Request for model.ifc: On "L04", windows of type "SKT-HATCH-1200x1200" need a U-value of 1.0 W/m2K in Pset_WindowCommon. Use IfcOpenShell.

First a look at what the model holds.

```python
import ifcopenshell
import ifcopenshell.util.element

model = ifcopenshell.open("model.ifc")
print(model.schema)
storey = next(s for s in model.by_type("IfcBuildingStorey") if s.Name == "L04")
windows = [e for e in ifcopenshell.util.element.get_decomposition(storey) if e.is_a("IfcWindow")]
seen = {}
for e in windows:
    element_type = ifcopenshell.util.element.get_type(e)
    key = (element_type.Name if element_type != e and element_type else None, ifcopenshell.util.element.get_pset(e, "Pset_WindowCommon", "ThermalTransmittance"))
    seen[key] = seen.get(key, 0) + 1
for (name, value), count in sorted(seen.items(), key=str):
    print(count, "x", name, "|", value)
```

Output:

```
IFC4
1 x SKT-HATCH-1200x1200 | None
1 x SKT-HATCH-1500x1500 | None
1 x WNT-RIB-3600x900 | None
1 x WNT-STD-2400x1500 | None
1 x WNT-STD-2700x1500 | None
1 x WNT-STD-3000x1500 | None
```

```python
import ifcopenshell
import ifcopenshell.api.pset
import ifcopenshell.util.element

model = ifcopenshell.open("model.ifc")

storey = next(s for s in model.by_type("IfcBuildingStorey") if s.Name == "L04")
windows = [e for e in ifcopenshell.util.element.get_decomposition(storey) if e.is_a("IfcWindow")]

count = 0
for e in windows:
    element_type = ifcopenshell.util.element.get_type(e)
    if element_type in (None, e) or element_type.Name != "SKT-HATCH-1200x1200":
        continue
    # add_pset returns the element's existing set when there is one.
    pset = ifcopenshell.api.pset.add_pset(model, product=e, name="Pset_WindowCommon")
    ifcopenshell.api.pset.edit_pset(model, pset=pset, properties={"ThermalTransmittance": 1.0})
    count += 1

print(count, "windows updated")

model.write("model-out.ifc")
```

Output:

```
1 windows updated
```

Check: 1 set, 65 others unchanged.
